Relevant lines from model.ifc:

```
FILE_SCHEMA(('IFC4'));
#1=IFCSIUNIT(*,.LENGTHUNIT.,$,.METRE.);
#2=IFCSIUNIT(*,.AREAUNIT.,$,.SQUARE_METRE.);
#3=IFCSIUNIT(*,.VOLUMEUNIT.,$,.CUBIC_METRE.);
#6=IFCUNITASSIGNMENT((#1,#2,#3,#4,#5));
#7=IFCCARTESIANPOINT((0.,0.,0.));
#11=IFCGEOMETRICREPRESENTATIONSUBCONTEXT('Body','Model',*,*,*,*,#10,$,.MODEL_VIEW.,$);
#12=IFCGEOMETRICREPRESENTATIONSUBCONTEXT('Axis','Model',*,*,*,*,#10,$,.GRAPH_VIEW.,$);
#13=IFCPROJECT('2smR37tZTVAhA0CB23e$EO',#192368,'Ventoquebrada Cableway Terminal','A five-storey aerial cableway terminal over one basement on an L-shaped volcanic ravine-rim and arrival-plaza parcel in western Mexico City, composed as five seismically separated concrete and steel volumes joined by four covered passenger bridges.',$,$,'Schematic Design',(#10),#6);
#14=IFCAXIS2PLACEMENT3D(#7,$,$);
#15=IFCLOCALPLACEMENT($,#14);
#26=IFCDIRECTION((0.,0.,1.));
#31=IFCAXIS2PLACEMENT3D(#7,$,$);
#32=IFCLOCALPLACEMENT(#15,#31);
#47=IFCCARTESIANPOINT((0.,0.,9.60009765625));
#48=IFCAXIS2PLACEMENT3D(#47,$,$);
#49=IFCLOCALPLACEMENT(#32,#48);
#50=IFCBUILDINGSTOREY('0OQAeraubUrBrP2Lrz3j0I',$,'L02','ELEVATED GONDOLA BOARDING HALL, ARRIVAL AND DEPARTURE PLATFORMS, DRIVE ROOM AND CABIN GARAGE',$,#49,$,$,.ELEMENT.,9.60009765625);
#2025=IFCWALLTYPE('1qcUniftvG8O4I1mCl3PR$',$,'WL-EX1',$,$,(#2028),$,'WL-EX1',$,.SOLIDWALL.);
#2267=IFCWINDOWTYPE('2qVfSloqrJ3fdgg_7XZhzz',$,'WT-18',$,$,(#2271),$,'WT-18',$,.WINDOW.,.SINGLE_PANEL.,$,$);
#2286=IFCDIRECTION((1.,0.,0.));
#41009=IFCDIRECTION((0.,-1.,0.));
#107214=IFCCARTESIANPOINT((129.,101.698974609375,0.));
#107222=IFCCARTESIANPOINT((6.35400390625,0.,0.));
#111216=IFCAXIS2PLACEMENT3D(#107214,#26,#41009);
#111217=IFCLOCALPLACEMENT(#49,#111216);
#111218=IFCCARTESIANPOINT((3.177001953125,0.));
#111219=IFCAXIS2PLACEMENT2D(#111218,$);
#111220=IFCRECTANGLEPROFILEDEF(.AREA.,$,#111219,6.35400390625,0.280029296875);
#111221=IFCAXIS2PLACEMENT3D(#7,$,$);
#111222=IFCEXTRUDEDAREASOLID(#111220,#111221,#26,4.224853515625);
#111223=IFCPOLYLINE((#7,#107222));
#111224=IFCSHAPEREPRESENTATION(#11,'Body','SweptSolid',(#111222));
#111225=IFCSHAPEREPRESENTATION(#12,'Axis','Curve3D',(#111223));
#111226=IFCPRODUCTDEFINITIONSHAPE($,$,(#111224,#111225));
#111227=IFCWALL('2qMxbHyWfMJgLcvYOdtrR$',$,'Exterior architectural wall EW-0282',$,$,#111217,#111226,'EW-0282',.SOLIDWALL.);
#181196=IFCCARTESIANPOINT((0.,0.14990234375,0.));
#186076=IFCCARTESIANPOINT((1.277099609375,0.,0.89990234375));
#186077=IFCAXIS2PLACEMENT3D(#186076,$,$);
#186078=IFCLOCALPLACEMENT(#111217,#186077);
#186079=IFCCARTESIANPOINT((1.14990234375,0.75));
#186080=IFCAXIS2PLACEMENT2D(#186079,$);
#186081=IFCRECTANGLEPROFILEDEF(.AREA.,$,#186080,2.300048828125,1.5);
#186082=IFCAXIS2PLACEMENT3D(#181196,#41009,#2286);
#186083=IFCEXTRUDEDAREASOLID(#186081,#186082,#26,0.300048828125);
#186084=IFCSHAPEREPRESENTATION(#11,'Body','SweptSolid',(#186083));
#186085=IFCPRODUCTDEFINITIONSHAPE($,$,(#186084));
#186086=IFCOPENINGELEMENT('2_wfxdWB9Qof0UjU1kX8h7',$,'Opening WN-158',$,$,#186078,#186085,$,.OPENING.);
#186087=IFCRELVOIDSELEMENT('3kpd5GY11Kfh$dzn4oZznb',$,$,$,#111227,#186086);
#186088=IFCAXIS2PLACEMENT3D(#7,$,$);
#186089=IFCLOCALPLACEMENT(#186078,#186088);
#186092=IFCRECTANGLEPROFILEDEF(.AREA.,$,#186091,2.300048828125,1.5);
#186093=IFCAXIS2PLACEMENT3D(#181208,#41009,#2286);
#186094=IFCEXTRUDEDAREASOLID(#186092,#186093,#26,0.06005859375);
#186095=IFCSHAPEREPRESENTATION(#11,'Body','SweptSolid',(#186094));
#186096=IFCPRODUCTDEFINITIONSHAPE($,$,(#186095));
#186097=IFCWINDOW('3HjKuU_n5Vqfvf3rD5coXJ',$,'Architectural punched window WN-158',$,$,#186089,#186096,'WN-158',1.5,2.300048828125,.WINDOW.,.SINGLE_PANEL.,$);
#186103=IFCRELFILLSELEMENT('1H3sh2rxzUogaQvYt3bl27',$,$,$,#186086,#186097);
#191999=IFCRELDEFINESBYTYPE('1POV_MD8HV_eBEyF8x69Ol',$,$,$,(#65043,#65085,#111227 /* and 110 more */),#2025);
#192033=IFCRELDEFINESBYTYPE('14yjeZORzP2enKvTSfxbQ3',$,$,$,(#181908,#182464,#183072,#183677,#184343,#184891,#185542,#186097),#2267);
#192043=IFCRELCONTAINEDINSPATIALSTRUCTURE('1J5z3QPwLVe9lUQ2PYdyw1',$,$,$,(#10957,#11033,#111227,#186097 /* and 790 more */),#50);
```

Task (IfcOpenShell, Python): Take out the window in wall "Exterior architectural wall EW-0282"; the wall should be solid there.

```python
import ifcopenshell
import ifcopenshell.api.feature
import ifcopenshell.api.root
import ifcopenshell.geom
import ifcopenshell.util.shape

model = ifcopenshell.open("model.ifc")
settings = ifcopenshell.geom.settings()


def volume(element):
    """Net volume in cubic metres, openings subtracted."""
    shape = ifcopenshell.geom.create_shape(settings, element)
    return ifcopenshell.util.shape.get_volume(shape.geometry)


window = model.by_guid("3HjKuU_n5Vqfvf3rD5coXJ")
opening = window.FillsVoids[0].RelatingOpeningElement
wall = opening.VoidsElements[0].RelatingBuildingElement
before = volume(wall)

ifcopenshell.api.root.remove_product(model, product=window)
ifcopenshell.api.feature.remove_feature(model, feature=opening)

after = volume(wall)

print(f"wall volume {before:.3f} -> {after:.3f} m3")

model.write("model_rev.ifc")
```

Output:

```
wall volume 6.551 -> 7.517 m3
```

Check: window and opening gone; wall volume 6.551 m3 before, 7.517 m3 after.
